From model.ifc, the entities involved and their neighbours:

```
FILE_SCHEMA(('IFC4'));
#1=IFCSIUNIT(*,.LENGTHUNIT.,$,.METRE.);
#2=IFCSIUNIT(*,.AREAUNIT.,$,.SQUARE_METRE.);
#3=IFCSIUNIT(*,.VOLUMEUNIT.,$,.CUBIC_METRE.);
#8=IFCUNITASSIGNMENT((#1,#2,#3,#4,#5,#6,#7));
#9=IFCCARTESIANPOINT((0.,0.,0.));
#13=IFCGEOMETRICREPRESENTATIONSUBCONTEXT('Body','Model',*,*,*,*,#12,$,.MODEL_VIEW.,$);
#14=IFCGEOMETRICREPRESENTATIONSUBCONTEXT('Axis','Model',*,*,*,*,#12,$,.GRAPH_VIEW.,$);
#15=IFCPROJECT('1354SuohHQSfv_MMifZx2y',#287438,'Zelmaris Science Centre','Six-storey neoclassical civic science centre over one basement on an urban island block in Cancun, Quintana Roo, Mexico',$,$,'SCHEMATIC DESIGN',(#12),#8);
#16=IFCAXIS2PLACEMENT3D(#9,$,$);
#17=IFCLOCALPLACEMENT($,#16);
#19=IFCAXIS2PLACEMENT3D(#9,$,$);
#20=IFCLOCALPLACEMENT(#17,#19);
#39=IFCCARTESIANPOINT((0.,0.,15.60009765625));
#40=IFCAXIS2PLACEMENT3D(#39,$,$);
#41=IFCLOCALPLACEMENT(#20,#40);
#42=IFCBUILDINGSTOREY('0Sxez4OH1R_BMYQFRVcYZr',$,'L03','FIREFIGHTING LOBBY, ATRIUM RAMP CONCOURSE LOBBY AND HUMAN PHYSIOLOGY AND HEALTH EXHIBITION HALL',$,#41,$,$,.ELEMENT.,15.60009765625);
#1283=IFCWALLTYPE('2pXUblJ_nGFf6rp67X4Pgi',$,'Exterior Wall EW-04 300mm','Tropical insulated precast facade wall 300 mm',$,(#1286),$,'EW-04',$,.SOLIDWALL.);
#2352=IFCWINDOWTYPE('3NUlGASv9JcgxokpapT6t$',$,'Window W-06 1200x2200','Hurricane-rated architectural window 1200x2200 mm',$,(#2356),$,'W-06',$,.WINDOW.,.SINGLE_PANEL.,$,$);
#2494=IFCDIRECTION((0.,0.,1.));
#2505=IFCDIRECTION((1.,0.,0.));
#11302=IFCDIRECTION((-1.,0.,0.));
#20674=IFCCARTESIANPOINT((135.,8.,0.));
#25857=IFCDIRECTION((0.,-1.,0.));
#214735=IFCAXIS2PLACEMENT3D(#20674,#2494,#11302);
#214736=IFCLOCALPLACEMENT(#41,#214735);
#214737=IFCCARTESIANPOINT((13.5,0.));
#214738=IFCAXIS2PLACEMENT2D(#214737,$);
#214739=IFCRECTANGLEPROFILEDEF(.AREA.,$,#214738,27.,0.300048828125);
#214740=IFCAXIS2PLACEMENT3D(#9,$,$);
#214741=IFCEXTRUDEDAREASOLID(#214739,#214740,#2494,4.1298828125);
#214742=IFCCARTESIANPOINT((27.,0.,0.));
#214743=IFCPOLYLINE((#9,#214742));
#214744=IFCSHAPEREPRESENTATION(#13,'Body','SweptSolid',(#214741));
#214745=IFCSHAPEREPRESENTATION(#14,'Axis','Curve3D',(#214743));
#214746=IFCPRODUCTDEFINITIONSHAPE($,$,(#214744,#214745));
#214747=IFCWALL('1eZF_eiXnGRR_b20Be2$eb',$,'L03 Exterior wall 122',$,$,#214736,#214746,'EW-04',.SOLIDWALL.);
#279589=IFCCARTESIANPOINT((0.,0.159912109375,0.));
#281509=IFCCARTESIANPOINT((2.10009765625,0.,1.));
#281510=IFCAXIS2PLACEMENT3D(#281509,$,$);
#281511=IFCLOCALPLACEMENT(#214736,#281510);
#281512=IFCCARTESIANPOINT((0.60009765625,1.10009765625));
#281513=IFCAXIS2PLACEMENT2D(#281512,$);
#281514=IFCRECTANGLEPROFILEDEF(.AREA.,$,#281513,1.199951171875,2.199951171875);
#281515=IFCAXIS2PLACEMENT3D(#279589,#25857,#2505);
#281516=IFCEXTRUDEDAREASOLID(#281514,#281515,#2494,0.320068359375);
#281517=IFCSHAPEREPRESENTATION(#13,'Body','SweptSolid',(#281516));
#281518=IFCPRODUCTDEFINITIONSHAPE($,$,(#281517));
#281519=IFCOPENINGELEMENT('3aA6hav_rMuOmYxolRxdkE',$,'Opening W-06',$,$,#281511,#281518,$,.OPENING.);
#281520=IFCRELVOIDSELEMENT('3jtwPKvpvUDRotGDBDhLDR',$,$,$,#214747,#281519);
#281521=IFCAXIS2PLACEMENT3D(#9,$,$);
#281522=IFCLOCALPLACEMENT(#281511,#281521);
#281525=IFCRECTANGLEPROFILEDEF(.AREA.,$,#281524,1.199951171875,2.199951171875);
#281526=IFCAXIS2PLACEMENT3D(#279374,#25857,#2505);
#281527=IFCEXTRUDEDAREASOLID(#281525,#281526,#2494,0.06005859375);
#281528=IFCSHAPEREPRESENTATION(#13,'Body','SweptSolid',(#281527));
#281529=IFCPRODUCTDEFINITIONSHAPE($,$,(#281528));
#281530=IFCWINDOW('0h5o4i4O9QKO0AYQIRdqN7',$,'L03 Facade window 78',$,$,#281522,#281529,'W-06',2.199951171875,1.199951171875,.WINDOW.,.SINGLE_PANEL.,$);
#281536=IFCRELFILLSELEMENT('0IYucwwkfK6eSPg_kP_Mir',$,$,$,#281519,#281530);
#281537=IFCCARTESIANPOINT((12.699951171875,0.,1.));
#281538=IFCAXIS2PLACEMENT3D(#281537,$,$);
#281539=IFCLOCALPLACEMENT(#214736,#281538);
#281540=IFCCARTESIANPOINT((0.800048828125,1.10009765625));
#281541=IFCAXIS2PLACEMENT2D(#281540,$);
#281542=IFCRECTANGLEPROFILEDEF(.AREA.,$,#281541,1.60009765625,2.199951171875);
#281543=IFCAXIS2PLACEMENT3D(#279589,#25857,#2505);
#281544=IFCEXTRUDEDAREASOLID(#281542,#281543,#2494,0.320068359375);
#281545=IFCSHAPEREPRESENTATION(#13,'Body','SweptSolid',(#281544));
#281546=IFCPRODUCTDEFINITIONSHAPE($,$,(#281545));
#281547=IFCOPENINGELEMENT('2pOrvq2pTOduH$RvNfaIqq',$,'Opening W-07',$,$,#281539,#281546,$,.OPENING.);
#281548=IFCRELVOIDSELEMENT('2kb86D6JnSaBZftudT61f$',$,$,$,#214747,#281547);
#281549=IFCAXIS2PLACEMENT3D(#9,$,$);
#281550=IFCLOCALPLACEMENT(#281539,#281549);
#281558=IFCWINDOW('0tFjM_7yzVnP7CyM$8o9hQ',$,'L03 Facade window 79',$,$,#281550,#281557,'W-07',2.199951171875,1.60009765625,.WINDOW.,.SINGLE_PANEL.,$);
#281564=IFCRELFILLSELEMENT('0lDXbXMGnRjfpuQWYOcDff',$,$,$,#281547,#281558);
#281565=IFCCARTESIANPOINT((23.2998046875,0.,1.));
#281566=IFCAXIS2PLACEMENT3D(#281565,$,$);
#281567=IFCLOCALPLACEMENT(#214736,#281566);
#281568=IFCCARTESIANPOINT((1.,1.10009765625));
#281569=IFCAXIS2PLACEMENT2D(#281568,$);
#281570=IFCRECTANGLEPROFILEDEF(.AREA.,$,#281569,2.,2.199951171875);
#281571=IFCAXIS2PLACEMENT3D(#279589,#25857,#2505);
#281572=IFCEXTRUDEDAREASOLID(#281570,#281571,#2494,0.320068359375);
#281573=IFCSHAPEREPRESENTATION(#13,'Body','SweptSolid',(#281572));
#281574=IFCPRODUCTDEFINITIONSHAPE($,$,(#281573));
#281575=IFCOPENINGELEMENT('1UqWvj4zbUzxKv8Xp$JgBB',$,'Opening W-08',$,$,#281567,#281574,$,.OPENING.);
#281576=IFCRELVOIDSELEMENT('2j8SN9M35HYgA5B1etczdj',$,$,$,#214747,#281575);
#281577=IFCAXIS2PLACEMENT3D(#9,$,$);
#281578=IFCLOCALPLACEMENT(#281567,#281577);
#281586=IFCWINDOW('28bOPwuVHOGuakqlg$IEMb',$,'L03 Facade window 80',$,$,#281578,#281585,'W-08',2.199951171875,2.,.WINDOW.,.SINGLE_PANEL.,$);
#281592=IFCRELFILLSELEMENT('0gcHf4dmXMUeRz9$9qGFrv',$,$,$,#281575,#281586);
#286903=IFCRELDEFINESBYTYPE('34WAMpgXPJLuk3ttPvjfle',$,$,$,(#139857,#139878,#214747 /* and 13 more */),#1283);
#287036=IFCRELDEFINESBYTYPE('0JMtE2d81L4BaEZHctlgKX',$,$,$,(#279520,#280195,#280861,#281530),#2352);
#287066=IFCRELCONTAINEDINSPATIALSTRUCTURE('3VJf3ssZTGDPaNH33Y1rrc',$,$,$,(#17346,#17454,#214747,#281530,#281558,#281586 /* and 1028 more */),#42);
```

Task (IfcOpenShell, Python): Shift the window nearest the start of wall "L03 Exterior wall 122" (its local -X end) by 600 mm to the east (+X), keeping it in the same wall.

```python
import ifcopenshell
import ifcopenshell.api.geometry
import ifcopenshell.util.placement
import ifcopenshell.util.unit

model = ifcopenshell.open("model.ifc")
unit_scale = ifcopenshell.util.unit.calculate_unit_scale(model)

window = model.by_guid("0h5o4i4O9QKO0AYQIRdqN7")
opening = window.FillsVoids[0].RelatingOpeningElement
wall = opening.VoidsElements[0].RelatingBuildingElement

wall_matrix = ifcopenshell.util.placement.get_local_placement(wall.ObjectPlacement)
shift = wall_matrix[:3, 0] * -0.6 / unit_scale
before = ifcopenshell.util.placement.get_local_placement(window.ObjectPlacement)[:3, 3].copy()

# The window is placed relative to its opening, so it follows when the opening moves.
matrix = ifcopenshell.util.placement.get_local_placement(opening.ObjectPlacement)
matrix[:3, 3] += shift
ifcopenshell.api.geometry.edit_object_placement(
    model, product=opening, matrix=matrix, is_si=False, should_transform_children=True
)

after = ifcopenshell.util.placement.get_local_placement(window.ObjectPlacement)[:3, 3]
print("window moved by", (after - before).round(3) + 0.0)

model.write("model_updated.ifc")
```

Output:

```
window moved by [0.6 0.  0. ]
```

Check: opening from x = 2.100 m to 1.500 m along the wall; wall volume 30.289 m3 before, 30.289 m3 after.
